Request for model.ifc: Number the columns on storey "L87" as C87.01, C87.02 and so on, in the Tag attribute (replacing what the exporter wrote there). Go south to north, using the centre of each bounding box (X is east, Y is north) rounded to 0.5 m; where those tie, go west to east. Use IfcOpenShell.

First a look at what the model holds.

```python
import ifcopenshell
import ifcopenshell.util.element
import ifcopenshell.util.placement

model = ifcopenshell.open("model.ifc")
print(model.schema)
storey = next(s for s in model.by_type("IfcBuildingStorey") if s.Name == "L87")
columns = [e for e in ifcopenshell.util.element.get_decomposition(storey) if e.is_a("IfcColumn")]
for e in sorted(columns, key=lambda e: e.id()):
    origin = ifcopenshell.util.placement.get_local_placement(e.ObjectPlacement)[:3, 3]
    print(e.id(), e.Tag, e.Name, origin.round(2) + 0.0, sep=" | ")
```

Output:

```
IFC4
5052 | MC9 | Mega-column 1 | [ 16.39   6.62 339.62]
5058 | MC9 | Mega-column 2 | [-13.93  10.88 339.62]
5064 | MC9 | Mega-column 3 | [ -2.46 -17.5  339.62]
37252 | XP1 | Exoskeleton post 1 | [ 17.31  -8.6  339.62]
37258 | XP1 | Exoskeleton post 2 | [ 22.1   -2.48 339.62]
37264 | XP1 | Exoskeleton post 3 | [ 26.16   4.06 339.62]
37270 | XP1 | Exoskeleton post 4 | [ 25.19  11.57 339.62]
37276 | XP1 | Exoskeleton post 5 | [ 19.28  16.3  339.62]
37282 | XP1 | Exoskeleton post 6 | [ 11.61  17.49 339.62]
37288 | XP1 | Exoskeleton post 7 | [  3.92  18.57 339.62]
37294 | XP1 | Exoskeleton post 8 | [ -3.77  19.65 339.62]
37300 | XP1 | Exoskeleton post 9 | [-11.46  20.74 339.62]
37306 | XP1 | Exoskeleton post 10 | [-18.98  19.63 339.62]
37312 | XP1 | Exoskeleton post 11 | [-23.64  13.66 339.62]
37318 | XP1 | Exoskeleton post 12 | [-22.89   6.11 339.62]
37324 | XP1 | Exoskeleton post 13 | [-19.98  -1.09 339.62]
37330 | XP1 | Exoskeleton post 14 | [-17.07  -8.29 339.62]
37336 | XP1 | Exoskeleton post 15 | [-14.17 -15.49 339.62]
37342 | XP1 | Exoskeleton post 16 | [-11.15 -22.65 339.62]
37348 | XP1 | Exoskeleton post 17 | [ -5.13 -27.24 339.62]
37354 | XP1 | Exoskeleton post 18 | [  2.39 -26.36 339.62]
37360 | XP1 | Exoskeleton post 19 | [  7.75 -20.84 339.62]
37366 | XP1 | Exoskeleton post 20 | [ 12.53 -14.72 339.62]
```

```python
import ifcopenshell
import ifcopenshell.geom
import ifcopenshell.util.element
import ifcopenshell.util.shape

model = ifcopenshell.open("model.ifc")
settings = ifcopenshell.geom.settings()
settings.set("use-world-coords", True)


def centre(element):
    shape = ifcopenshell.geom.create_shape(settings, element)
    return ifcopenshell.util.shape.get_bbox_centroid(shape.geometry)


storey = next(s for s in model.by_type("IfcBuildingStorey") if s.Name == "L87")
columns = [e for e in ifcopenshell.util.element.get_decomposition(storey) if e.is_a("IfcColumn")]

# Insertion points can sit at a corner or the storey origin, so sort by the geometry (in metres).
centres = {e: centre(e) for e in columns}
columns.sort(key=lambda e: (round(centres[e][1] / 0.5), centres[e][0]))

for i, e in enumerate(columns, start=1):
    number = f"C87.{i:02d}"
    e.Tag = number
    print(e.id(), number)

model.write("model_rev.ifc")
```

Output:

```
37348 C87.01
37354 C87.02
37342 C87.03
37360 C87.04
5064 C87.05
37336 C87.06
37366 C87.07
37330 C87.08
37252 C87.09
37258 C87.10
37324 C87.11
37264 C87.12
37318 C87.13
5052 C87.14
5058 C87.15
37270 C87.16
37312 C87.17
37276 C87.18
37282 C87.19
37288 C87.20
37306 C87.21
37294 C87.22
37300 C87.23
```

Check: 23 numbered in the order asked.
